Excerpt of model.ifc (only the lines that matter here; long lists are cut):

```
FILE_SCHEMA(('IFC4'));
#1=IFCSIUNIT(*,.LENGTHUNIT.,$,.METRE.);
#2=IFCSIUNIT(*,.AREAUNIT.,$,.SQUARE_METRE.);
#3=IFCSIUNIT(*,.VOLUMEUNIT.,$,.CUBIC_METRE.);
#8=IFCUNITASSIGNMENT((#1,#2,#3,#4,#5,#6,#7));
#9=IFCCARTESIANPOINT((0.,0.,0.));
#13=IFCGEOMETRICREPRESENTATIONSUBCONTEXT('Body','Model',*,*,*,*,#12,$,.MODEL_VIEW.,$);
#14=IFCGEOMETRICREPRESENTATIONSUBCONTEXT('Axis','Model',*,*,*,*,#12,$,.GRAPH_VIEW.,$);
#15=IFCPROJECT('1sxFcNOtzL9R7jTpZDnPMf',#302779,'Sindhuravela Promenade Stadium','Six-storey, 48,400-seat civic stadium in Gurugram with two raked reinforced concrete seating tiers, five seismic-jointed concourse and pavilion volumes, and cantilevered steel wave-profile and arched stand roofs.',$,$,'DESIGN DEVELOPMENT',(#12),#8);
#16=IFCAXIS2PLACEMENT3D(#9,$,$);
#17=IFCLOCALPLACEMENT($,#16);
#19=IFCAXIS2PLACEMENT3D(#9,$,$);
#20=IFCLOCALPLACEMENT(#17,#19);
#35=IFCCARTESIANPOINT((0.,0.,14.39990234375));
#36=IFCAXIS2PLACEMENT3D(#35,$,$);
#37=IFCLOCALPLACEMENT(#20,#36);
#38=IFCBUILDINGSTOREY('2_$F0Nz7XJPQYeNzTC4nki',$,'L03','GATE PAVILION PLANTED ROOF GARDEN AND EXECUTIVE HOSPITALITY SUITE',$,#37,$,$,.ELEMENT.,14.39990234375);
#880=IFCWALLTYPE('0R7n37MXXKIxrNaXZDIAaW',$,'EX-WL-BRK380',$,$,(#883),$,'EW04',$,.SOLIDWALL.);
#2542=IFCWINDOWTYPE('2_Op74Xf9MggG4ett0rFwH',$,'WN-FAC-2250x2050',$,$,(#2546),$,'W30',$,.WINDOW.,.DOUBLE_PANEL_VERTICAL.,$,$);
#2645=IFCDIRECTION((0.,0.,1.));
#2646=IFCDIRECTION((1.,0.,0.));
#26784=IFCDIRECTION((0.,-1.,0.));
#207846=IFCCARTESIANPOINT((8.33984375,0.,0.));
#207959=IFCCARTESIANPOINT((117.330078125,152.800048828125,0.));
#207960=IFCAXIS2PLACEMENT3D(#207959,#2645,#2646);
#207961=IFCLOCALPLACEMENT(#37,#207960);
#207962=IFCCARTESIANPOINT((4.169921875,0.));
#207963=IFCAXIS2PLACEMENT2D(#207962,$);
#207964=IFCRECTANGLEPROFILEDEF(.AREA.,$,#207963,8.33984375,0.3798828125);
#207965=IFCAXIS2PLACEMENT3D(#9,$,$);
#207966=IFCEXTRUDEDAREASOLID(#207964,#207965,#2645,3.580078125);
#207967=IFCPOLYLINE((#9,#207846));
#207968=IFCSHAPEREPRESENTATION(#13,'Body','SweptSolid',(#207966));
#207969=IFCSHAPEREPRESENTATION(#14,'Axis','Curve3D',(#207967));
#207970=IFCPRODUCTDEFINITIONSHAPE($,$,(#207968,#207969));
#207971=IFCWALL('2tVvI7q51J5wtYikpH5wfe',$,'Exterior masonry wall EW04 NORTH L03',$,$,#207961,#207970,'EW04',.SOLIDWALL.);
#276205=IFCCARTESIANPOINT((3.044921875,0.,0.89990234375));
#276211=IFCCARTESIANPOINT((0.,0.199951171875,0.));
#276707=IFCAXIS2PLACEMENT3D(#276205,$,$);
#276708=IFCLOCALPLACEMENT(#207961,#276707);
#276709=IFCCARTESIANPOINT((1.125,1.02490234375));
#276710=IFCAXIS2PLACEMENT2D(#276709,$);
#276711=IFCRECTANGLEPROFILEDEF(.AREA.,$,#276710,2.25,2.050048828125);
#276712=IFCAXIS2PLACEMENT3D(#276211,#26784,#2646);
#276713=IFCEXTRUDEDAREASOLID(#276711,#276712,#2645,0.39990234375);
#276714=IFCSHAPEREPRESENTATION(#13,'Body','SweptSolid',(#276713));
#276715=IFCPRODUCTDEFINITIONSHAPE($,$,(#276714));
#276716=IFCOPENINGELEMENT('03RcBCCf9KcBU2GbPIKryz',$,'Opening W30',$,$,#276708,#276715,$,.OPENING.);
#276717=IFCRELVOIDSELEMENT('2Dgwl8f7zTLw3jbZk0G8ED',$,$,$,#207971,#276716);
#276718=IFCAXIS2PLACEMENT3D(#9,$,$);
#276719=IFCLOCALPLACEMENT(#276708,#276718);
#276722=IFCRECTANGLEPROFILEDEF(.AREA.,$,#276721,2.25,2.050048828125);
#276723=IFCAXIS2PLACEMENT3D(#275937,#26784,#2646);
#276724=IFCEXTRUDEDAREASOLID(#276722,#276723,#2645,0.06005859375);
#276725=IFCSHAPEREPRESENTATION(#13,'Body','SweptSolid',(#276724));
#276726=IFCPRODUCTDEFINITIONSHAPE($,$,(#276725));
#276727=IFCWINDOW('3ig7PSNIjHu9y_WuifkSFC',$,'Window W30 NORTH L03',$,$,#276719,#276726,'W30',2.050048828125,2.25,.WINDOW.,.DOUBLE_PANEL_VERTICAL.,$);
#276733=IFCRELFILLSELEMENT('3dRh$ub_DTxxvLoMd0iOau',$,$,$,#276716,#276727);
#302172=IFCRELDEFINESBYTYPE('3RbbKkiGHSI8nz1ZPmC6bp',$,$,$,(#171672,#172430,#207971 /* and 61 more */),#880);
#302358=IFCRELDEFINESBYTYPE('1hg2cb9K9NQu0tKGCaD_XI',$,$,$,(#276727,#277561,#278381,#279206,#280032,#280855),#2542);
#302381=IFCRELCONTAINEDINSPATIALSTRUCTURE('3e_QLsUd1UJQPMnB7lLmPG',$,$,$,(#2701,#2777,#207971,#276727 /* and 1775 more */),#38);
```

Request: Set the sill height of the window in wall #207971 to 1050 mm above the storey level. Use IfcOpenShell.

```python
import numpy as np
import ifcopenshell
import ifcopenshell.api.geometry
import ifcopenshell.geom
import ifcopenshell.util.element
import ifcopenshell.util.placement
import ifcopenshell.util.shape
import ifcopenshell.util.unit

model = ifcopenshell.open("model.ifc")
unit_scale = ifcopenshell.util.unit.calculate_unit_scale(model)

window = model.by_guid("3ig7PSNIjHu9y_WuifkSFC")
opening = window.FillsVoids[0].RelatingOpeningElement
storey = ifcopenshell.util.element.get_container(window, ifc_class="IfcBuildingStorey")
level = ifcopenshell.util.placement.get_local_placement(storey.ObjectPlacement)[2, 3]

# The opening's origin need not be at the sill, so measure its lowest point.
shape = ifcopenshell.geom.create_shape(ifcopenshell.geom.settings(), opening)
bottom = ifcopenshell.util.shape.get_shape_bottom_elevation(shape, shape.geometry) / unit_scale
dz = level + 1.05 / unit_scale - bottom

shift = np.array([0.0, 0.0, dz])
# The window is placed relative to its opening, so it follows when the opening moves.
matrix = ifcopenshell.util.placement.get_local_placement(opening.ObjectPlacement)
matrix[:3, 3] += shift
ifcopenshell.api.geometry.edit_object_placement(
    model, product=opening, matrix=matrix, is_si=False, should_transform_children=True
)

print(f"moved by {dz * unit_scale:+.3f} m")

model.write("model_edited.ifc")
```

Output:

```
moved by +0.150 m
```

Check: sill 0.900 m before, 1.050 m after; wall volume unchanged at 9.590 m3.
